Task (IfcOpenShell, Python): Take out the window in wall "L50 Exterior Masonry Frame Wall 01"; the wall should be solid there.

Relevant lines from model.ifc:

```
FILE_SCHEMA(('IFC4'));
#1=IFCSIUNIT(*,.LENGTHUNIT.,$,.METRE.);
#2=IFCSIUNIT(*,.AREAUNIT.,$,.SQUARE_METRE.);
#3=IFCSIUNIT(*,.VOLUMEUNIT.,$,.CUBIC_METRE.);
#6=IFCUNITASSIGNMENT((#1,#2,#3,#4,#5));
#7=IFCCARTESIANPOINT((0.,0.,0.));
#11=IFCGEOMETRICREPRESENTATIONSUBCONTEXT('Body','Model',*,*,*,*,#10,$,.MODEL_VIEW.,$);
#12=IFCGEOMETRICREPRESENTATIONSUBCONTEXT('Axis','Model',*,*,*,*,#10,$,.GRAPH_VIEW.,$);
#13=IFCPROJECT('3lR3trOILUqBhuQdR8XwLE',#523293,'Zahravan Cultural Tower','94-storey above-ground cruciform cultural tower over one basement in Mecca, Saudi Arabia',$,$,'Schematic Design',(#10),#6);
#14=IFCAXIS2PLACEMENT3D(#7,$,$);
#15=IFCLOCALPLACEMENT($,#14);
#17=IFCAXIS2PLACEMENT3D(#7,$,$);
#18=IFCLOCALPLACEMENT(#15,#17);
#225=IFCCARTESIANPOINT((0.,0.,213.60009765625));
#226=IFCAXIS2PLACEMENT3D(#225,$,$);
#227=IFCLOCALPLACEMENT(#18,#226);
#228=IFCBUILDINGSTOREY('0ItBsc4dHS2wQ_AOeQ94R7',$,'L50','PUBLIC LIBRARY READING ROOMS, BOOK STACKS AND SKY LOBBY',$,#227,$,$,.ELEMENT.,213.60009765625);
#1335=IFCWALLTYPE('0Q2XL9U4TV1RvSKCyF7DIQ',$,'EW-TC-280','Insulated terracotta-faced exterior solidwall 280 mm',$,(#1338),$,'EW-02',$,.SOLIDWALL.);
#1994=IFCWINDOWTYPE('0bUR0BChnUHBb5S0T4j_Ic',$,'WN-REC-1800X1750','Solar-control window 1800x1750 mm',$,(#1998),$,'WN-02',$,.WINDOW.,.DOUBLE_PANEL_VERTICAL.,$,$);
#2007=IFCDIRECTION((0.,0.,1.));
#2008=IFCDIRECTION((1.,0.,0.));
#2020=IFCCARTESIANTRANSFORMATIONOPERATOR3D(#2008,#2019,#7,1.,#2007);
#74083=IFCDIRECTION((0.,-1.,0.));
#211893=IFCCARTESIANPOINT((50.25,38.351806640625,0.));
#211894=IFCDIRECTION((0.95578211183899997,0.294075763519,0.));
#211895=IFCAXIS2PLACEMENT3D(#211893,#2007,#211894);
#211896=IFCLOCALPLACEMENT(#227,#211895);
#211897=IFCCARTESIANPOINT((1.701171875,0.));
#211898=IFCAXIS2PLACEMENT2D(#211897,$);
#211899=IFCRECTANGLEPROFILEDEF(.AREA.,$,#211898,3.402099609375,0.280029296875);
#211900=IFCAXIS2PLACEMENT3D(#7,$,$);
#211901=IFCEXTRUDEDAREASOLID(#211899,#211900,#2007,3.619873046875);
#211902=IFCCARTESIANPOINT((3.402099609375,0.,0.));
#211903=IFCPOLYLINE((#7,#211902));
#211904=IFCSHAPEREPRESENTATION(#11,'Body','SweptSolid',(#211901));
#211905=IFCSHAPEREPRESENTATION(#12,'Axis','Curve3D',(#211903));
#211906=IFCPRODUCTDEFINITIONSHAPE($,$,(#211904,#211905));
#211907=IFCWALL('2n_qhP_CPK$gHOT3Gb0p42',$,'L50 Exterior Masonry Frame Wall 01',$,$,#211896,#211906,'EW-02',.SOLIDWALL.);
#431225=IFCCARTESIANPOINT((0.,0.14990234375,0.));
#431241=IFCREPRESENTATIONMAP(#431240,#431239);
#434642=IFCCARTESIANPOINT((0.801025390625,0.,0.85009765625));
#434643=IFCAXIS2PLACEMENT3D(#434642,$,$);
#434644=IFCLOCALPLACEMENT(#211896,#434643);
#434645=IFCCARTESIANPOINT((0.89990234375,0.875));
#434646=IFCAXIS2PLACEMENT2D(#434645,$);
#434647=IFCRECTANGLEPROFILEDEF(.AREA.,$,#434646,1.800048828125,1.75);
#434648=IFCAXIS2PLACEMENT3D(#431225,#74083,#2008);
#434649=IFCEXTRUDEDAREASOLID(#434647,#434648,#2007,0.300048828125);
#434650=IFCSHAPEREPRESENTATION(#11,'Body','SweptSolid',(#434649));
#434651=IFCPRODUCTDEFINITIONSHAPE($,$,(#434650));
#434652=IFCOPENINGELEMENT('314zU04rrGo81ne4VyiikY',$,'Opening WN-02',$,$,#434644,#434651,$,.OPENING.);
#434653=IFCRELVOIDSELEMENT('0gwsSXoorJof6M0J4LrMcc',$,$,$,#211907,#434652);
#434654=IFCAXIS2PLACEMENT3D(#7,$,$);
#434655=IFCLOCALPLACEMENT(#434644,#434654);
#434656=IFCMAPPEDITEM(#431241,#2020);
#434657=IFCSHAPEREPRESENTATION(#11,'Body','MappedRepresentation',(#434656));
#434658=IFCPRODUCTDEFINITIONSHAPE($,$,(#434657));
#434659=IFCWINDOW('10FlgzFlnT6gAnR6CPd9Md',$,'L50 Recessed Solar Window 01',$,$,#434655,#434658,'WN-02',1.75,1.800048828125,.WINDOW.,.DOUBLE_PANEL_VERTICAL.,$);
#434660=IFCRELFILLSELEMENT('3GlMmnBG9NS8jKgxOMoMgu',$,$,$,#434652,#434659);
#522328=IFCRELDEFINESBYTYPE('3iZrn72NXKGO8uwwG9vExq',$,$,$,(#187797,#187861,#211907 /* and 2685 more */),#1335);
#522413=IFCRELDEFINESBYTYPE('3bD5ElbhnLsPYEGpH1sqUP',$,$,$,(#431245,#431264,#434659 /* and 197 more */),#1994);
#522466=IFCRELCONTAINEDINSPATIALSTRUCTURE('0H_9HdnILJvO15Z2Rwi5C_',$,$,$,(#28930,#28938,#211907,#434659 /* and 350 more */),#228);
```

```python
import ifcopenshell
import ifcopenshell.api.feature
import ifcopenshell.api.root
import ifcopenshell.geom
import ifcopenshell.util.shape

model = ifcopenshell.open("model.ifc")
settings = ifcopenshell.geom.settings()


def volume(element):
    """Net volume in cubic metres, openings subtracted."""
    shape = ifcopenshell.geom.create_shape(settings, element)
    return ifcopenshell.util.shape.get_volume(shape.geometry)


window = model.by_guid("10FlgzFlnT6gAnR6CPd9Md")
opening = window.FillsVoids[0].RelatingOpeningElement
wall = opening.VoidsElements[0].RelatingBuildingElement
before = volume(wall)

ifcopenshell.api.root.remove_product(model, product=window)
ifcopenshell.api.feature.remove_feature(model, feature=opening)

after = volume(wall)

print(f"wall volume {before:.3f} -> {after:.3f} m3")

model.write("model_rev.ifc")
```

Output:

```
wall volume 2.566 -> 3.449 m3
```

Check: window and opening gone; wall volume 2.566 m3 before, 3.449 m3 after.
